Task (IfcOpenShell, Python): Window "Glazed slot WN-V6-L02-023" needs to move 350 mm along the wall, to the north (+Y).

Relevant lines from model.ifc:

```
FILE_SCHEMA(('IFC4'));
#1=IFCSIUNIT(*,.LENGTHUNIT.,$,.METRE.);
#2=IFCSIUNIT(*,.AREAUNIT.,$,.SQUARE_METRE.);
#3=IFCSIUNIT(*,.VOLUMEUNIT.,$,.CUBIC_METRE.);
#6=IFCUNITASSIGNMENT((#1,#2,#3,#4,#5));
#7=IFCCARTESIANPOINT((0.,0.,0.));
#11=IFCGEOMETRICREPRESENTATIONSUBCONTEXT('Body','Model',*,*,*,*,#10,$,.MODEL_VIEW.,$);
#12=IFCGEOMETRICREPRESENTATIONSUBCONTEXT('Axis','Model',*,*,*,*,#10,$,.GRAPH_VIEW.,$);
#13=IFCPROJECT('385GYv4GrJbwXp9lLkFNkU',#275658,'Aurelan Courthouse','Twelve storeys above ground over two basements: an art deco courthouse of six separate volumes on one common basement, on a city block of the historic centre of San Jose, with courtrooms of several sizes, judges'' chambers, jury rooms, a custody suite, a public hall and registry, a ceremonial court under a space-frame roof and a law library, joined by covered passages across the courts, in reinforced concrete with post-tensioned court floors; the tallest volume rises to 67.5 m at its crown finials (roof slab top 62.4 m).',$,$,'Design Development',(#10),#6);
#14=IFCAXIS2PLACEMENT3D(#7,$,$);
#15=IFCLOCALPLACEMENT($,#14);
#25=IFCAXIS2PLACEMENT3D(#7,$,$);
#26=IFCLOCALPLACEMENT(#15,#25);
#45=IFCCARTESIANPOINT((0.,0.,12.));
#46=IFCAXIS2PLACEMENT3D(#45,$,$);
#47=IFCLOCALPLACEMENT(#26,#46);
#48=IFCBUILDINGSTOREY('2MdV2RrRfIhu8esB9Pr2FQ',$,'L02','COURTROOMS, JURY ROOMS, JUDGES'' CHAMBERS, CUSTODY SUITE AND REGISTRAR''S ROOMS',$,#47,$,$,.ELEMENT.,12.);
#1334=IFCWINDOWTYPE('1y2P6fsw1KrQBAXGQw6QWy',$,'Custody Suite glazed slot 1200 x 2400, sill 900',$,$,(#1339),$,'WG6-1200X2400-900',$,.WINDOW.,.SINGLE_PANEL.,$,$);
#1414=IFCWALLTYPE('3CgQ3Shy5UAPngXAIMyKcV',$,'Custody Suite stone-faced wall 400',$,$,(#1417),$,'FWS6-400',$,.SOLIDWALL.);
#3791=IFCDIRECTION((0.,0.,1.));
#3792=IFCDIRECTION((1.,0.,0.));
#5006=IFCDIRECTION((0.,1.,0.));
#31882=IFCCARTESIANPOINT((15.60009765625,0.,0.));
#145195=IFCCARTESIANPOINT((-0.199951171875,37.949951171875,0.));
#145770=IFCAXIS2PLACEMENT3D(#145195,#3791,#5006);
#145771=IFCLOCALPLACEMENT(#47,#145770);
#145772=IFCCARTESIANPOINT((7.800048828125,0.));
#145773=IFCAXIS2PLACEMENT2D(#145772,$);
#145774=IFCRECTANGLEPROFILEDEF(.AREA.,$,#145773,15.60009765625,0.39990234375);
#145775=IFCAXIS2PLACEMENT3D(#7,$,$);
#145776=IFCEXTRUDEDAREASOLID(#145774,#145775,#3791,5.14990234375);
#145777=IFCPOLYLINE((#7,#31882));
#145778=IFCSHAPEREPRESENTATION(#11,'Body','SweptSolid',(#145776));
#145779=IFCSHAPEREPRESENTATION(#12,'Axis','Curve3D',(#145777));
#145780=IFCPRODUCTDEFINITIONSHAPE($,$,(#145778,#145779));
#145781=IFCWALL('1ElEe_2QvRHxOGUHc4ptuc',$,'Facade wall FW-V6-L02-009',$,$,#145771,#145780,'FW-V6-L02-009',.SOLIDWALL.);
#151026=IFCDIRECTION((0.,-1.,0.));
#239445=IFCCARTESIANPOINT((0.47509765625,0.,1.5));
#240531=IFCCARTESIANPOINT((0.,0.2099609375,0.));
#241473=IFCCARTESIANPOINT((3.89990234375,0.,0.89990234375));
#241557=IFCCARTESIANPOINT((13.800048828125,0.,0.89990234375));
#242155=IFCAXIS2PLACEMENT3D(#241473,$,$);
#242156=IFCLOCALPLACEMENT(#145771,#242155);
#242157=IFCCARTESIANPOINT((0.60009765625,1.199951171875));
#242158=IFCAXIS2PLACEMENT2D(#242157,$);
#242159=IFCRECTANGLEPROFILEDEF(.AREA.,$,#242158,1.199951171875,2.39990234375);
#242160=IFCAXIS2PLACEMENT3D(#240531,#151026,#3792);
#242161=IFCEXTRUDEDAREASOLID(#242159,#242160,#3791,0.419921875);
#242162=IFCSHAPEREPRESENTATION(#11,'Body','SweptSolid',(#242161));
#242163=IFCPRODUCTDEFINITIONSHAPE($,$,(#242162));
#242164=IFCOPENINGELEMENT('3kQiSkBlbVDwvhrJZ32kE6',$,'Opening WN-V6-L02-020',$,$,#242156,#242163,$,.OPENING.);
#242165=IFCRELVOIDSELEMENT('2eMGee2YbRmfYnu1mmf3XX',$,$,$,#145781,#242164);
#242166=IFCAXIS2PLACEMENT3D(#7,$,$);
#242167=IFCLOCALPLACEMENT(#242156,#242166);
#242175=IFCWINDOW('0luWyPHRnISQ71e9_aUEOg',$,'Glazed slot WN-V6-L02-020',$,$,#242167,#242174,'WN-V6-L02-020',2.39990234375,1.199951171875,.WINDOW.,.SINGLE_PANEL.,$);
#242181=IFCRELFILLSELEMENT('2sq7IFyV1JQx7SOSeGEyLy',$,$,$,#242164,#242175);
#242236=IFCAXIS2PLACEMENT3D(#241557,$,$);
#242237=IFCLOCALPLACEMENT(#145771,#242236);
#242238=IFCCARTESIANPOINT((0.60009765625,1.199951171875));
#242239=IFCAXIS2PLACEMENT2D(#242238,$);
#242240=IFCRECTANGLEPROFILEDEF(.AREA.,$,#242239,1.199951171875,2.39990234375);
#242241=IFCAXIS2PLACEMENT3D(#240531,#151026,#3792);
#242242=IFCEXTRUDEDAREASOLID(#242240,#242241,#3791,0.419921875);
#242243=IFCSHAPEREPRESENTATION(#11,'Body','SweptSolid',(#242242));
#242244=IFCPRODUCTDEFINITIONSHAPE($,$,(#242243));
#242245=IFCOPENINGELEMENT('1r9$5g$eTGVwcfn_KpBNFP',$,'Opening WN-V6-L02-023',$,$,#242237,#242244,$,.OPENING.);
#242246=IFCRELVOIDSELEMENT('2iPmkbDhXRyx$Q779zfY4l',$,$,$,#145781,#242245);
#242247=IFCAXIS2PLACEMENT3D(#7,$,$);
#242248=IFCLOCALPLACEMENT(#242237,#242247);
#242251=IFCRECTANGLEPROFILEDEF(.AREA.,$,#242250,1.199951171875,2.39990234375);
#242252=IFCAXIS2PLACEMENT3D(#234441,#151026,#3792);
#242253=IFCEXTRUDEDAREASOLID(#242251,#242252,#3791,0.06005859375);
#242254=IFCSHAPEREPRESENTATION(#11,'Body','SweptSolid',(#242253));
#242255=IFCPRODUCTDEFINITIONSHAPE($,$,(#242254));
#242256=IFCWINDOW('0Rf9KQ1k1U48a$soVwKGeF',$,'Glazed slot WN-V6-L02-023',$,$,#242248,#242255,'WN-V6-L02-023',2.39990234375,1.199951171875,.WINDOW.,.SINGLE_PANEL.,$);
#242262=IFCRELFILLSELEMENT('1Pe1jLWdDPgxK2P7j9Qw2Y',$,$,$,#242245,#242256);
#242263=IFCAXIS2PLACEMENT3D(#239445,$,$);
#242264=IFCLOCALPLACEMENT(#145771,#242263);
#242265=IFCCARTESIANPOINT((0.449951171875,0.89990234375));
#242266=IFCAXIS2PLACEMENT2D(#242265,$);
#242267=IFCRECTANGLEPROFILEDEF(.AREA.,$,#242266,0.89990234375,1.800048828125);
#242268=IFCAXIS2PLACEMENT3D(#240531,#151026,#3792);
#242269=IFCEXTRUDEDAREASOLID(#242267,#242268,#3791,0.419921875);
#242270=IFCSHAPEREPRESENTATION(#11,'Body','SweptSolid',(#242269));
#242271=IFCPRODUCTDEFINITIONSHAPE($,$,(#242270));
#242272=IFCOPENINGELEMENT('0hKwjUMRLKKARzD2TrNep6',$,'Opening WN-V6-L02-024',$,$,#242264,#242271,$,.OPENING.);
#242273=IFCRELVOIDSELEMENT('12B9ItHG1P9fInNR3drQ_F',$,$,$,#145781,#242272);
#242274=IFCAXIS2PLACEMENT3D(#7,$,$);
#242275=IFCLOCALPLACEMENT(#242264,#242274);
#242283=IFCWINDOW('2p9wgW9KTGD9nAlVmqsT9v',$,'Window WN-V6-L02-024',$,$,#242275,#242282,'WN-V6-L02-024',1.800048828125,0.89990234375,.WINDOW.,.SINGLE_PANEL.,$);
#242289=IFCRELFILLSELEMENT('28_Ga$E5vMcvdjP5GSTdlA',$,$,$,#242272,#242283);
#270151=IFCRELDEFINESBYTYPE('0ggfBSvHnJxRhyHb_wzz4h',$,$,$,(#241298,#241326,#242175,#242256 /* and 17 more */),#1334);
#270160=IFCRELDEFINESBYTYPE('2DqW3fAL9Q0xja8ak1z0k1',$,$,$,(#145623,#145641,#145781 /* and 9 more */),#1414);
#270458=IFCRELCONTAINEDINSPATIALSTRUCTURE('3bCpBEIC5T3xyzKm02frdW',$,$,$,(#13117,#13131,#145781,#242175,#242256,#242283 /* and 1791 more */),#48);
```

```python
import ifcopenshell
import ifcopenshell.api.geometry
import ifcopenshell.util.placement
import ifcopenshell.util.unit

model = ifcopenshell.open("model.ifc")
unit_scale = ifcopenshell.util.unit.calculate_unit_scale(model)

window = model.by_guid("0Rf9KQ1k1U48a$soVwKGeF")
opening = window.FillsVoids[0].RelatingOpeningElement
wall = opening.VoidsElements[0].RelatingBuildingElement

wall_matrix = ifcopenshell.util.placement.get_local_placement(wall.ObjectPlacement)
shift = wall_matrix[:3, 0] * 0.35 / unit_scale
before = ifcopenshell.util.placement.get_local_placement(window.ObjectPlacement)[:3, 3].copy()

# The window is placed relative to its opening, so it follows when the opening moves.
matrix = ifcopenshell.util.placement.get_local_placement(opening.ObjectPlacement)
matrix[:3, 3] += shift
ifcopenshell.api.geometry.edit_object_placement(
    model, product=opening, matrix=matrix, is_si=False, should_transform_children=True
)

after = ifcopenshell.util.placement.get_local_placement(window.ObjectPlacement)[:3, 3]
print("window moved by", (after - before).round(3) + 0.0)

model.write("model-out.ifc")
```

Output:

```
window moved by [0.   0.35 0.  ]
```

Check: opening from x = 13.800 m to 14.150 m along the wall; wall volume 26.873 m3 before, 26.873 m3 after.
